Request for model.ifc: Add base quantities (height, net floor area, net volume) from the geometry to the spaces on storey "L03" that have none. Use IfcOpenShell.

First a look at what the model holds.

```python
import ifcopenshell
import ifcopenshell.util.element
import ifcopenshell.util.unit

model = ifcopenshell.open("model.ifc")
print(model.schema)
for unit_type in ("LENGTHUNIT", "AREAUNIT", "VOLUMEUNIT"):
    print(unit_type, ifcopenshell.util.unit.calculate_unit_scale(model, unit_type))
storey = next(s for s in model.by_type("IfcBuildingStorey") if s.Name == "L03")
spaces = [e for e in ifcopenshell.util.element.get_decomposition(storey) if e.is_a("IfcSpace")]
for e in sorted(spaces, key=lambda e: e.id()):
    print(e.id(), e.is_a(), e.Name, list(ifcopenshell.util.element.get_psets(e, qtos_only=True)), sep=" | ")
```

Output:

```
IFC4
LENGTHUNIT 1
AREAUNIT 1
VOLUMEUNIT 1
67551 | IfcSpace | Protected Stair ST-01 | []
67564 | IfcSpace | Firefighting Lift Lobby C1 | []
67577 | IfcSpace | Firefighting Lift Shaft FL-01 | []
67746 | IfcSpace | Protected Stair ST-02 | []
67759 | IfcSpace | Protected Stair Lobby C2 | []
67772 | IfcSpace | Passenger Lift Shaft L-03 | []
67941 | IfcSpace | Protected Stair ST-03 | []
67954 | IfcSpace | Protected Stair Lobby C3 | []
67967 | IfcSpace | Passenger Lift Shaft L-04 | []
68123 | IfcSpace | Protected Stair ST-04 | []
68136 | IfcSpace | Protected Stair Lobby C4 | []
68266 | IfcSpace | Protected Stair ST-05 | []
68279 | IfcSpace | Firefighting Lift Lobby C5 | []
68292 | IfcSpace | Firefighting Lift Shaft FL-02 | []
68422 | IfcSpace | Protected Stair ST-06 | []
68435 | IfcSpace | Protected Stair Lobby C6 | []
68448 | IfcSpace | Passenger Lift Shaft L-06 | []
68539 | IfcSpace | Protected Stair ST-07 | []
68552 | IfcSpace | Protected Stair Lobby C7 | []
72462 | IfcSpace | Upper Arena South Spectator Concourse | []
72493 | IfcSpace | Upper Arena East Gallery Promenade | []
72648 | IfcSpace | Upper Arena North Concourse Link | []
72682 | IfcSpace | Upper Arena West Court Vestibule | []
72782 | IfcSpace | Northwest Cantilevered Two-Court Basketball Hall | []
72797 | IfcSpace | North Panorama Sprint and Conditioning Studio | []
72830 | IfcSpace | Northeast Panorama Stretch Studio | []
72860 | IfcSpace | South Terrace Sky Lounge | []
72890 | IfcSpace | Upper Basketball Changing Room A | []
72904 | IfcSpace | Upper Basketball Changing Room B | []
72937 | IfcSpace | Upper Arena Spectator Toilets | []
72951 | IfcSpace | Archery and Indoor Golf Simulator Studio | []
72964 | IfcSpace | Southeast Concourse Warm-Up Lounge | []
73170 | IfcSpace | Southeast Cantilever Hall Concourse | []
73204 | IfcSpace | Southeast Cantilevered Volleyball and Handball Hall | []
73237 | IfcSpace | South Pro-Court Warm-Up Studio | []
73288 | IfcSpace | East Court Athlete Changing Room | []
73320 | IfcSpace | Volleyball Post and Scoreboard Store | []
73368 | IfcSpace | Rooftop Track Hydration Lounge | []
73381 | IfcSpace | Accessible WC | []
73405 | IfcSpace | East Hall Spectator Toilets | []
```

```python
import ifcopenshell
import ifcopenshell.api.pset
import ifcopenshell.geom
import ifcopenshell.util.element
import ifcopenshell.util.shape
import ifcopenshell.util.unit

model = ifcopenshell.open("model.ifc")
unit_scale = ifcopenshell.util.unit.calculate_unit_scale(model)
area_scale = ifcopenshell.util.unit.calculate_unit_scale(model, "AREAUNIT")
volume_scale = ifcopenshell.util.unit.calculate_unit_scale(model, "VOLUMEUNIT")
settings = ifcopenshell.geom.settings()

storey = next(s for s in model.by_type("IfcBuildingStorey") if s.Name == "L03")
spaces = [e for e in ifcopenshell.util.element.get_decomposition(storey) if e.is_a("IfcSpace")]

for e in sorted(spaces, key=lambda e: e.id()):
    if ifcopenshell.util.element.get_psets(e, qtos_only=True, should_inherit=False):
        continue
    # Geometry comes back in metres, in the element's own axes.
    shape = ifcopenshell.geom.create_shape(settings, e)
    values = {
        "Height": ifcopenshell.util.shape.get_z(shape.geometry) / unit_scale,
        "NetFloorArea": ifcopenshell.util.shape.get_footprint_area(shape.geometry) / area_scale,
        "NetVolume": ifcopenshell.util.shape.get_volume(shape.geometry) / volume_scale,
    }
    qto = ifcopenshell.api.pset.add_qto(model, product=e, name="Qto_SpaceBaseQuantities")
    ifcopenshell.api.pset.edit_qto(model, qto=qto, properties=values)
    print(e.id(), {k: round(v, 3) for k, v in values.items()})

model.write("model_updated.ifc")
```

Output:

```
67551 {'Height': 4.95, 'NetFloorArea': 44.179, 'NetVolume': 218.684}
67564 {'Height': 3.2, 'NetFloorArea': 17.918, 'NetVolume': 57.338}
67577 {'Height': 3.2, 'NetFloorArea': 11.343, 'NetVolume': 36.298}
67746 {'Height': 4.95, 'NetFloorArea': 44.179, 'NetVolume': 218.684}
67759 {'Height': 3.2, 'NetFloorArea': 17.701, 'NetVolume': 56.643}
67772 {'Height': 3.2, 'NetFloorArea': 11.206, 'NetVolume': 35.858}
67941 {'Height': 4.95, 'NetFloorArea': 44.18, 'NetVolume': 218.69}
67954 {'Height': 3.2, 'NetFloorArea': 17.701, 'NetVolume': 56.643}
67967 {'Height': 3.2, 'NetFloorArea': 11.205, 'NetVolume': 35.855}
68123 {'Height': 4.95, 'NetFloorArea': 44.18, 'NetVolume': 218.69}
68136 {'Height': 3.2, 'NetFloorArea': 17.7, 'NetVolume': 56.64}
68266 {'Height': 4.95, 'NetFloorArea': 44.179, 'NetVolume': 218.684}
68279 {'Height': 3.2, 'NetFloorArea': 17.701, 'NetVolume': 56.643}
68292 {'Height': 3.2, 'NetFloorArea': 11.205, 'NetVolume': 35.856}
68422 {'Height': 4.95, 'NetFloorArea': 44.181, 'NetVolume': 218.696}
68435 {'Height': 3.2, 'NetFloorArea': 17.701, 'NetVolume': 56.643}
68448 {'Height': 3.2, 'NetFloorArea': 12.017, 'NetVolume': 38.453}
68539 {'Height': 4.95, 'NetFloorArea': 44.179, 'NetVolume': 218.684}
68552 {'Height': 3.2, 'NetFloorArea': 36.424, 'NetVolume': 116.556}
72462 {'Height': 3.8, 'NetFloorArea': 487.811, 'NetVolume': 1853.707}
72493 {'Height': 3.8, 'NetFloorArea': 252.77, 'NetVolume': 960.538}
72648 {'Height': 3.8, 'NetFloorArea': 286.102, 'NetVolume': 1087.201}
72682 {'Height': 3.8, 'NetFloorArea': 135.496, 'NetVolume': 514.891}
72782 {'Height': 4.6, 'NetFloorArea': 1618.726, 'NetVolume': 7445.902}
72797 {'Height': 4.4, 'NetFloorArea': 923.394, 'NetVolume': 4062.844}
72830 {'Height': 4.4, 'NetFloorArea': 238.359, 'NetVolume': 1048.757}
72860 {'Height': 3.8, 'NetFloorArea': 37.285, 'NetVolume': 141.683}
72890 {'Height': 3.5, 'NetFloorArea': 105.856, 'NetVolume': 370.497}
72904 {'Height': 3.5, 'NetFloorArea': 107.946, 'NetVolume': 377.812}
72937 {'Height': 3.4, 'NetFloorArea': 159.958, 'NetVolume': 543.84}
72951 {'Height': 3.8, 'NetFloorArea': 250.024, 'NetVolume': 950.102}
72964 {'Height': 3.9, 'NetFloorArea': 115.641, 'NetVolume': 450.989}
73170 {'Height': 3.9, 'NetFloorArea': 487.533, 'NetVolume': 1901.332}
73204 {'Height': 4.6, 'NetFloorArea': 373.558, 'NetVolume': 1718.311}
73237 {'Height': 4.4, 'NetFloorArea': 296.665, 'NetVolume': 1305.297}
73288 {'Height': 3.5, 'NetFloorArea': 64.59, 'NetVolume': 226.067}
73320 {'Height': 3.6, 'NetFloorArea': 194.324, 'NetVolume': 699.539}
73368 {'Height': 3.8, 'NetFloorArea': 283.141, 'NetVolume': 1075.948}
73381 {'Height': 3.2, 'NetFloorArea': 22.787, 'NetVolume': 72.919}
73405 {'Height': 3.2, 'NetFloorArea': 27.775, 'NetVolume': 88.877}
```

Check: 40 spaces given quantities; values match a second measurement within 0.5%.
